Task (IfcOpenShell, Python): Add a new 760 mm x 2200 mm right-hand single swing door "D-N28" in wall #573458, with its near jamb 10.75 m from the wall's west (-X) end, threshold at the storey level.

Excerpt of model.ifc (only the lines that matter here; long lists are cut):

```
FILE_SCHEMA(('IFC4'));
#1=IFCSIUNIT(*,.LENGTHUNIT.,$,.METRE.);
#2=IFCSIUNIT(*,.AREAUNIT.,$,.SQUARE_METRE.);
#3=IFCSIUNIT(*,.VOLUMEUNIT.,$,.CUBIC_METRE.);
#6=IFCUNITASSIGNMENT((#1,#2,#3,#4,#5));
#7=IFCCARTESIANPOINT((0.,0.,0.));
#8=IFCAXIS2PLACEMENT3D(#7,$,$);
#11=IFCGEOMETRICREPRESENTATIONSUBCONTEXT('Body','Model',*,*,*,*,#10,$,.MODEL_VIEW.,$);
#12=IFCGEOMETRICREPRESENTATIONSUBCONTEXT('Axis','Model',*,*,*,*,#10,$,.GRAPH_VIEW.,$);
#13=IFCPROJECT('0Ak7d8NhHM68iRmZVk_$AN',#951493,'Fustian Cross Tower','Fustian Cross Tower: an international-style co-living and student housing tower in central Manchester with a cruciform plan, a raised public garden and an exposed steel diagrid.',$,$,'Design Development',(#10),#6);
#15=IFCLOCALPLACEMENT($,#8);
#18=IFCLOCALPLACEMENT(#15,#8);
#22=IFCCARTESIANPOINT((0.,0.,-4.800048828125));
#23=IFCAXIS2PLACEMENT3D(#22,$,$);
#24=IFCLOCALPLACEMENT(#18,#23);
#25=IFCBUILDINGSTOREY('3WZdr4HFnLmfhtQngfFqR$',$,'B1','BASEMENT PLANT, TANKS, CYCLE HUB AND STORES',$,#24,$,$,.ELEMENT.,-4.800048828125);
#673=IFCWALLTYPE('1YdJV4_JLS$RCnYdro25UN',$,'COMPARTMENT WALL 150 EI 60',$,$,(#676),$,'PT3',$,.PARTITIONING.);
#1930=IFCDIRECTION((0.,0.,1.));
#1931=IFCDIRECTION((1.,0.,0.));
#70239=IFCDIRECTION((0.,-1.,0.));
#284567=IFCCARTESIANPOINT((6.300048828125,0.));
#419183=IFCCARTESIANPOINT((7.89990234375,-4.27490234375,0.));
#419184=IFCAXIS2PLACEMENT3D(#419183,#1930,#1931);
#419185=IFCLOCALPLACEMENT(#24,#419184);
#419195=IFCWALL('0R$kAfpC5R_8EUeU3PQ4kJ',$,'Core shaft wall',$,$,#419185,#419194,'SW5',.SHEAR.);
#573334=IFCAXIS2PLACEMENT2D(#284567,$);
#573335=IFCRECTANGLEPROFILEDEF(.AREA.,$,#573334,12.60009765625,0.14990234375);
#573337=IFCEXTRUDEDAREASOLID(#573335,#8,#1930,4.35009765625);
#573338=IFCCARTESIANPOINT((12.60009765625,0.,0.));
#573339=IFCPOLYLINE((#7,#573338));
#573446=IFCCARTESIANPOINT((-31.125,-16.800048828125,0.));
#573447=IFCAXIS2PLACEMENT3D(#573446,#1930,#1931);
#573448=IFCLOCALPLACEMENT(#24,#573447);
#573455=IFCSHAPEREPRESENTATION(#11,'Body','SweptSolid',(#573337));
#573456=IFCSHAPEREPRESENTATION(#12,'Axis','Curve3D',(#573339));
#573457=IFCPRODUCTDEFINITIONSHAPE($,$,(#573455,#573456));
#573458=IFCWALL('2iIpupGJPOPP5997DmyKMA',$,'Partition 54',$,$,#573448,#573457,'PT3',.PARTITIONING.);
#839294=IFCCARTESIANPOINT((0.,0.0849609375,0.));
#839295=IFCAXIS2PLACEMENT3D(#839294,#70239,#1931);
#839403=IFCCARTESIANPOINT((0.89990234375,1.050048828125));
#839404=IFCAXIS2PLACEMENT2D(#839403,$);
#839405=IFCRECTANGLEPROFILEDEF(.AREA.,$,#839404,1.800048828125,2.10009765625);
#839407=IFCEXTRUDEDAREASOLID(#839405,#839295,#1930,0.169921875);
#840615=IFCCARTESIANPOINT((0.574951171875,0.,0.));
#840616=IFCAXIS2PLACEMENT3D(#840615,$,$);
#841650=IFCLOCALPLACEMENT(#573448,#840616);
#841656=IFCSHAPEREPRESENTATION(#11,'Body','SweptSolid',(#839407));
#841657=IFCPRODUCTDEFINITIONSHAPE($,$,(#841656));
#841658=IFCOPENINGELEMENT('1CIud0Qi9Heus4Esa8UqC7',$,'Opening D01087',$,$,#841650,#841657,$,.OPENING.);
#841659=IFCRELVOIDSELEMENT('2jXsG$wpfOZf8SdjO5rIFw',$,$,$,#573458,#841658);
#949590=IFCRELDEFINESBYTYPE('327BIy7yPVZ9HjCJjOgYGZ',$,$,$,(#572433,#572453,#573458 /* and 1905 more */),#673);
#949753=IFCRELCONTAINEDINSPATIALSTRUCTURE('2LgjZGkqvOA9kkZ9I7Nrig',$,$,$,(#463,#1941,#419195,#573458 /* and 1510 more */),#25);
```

```python
import numpy as np
import ifcopenshell
import ifcopenshell.api.feature
import ifcopenshell.api.geometry
import ifcopenshell.api.root
import ifcopenshell.api.spatial
import ifcopenshell.geom
import ifcopenshell.util.element
import ifcopenshell.util.placement
import ifcopenshell.util.representation
import ifcopenshell.util.shape
import ifcopenshell.util.unit

model = ifcopenshell.open("model.ifc")
unit_scale = ifcopenshell.util.unit.calculate_unit_scale(model)
settings = ifcopenshell.geom.settings()


def volume(element):
    """Net volume in cubic metres, openings subtracted."""
    shape = ifcopenshell.geom.create_shape(settings, element)
    return ifcopenshell.util.shape.get_volume(shape.geometry)


wall = model.by_id(573458)
storey = ifcopenshell.util.element.get_container(wall, ifc_class="IfcBuildingStorey")
context = ifcopenshell.util.representation.get_context(model, "Model", "Body", "MODEL_VIEW")
before = volume(wall)

width, height, from_end, sill = 0.76, 2.2, 10.75, 0.0  # metres

# The wall runs along its own X axis, and the end named is its -X end.
wall_shape = ifcopenshell.geom.create_shape(settings, wall)
x, y, z = ifcopenshell.util.shape.get_vertices(wall_shape.geometry).T
start = x.min() + from_end
face, thickness = float(y.min()), float(y.max() - y.min())
wall_matrix = ifcopenshell.util.placement.get_local_placement(wall.ObjectPlacement)
level = ifcopenshell.util.placement.get_local_placement(storey.ObjectPlacement)[2, 3]


def in_wall(x, y):
    """Placement at x, y metres in the wall's axes, at sill height."""
    matrix = wall_matrix.copy()
    matrix[:, 3] = wall_matrix @ np.array([x / unit_scale, y / unit_scale, 0.0, 1.0])
    matrix[2, 3] = level + sill / unit_scale
    return matrix


# Opening: a box that overshoots both wall faces by 50 mm.
opening = ifcopenshell.api.root.create_entity(model, ifc_class="IfcOpeningElement", predefined_type="OPENING")
box = ifcopenshell.api.geometry.add_wall_representation(
    model, context=context, length=width, height=height, thickness=thickness + 0.1
)
ifcopenshell.api.geometry.assign_representation(model, product=opening, representation=box)
ifcopenshell.api.geometry.edit_object_placement(model, product=opening, matrix=in_wall(start, face - 0.05), is_si=False)
ifcopenshell.api.feature.add_feature(model, feature=opening, element=wall)

door = ifcopenshell.api.root.create_entity(model, ifc_class="IfcDoor", name="D-N28", predefined_type="DOOR")
door.OverallWidth, door.OverallHeight = width / unit_scale, height / unit_scale
door.OperationType = "SINGLE_SWING_RIGHT"
body = ifcopenshell.api.geometry.add_door_representation(
    model,
    context=context,
    overall_width=door.OverallWidth,
    overall_height=door.OverallHeight,
    operation_type="SINGLE_SWING_RIGHT",
    lining_properties={"LiningDepth": thickness / unit_scale, "ThresholdDepth": thickness / unit_scale},
)
ifcopenshell.api.geometry.assign_representation(model, product=door, representation=body)
ifcopenshell.api.spatial.assign_container(model, products=[door], relating_structure=storey)
ifcopenshell.api.feature.add_filling(model, opening=opening, element=door)

# The lining spans the wall, so the door starts at the wall face.
ifcopenshell.api.geometry.edit_object_placement(model, product=door, matrix=in_wall(start, face), is_si=False)

after = volume(wall)

print(f"wall volume {before:.3f} -> {after:.3f} m3")

model.write("model_updated.ifc")
```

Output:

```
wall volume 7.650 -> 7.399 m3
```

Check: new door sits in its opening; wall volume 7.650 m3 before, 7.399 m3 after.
